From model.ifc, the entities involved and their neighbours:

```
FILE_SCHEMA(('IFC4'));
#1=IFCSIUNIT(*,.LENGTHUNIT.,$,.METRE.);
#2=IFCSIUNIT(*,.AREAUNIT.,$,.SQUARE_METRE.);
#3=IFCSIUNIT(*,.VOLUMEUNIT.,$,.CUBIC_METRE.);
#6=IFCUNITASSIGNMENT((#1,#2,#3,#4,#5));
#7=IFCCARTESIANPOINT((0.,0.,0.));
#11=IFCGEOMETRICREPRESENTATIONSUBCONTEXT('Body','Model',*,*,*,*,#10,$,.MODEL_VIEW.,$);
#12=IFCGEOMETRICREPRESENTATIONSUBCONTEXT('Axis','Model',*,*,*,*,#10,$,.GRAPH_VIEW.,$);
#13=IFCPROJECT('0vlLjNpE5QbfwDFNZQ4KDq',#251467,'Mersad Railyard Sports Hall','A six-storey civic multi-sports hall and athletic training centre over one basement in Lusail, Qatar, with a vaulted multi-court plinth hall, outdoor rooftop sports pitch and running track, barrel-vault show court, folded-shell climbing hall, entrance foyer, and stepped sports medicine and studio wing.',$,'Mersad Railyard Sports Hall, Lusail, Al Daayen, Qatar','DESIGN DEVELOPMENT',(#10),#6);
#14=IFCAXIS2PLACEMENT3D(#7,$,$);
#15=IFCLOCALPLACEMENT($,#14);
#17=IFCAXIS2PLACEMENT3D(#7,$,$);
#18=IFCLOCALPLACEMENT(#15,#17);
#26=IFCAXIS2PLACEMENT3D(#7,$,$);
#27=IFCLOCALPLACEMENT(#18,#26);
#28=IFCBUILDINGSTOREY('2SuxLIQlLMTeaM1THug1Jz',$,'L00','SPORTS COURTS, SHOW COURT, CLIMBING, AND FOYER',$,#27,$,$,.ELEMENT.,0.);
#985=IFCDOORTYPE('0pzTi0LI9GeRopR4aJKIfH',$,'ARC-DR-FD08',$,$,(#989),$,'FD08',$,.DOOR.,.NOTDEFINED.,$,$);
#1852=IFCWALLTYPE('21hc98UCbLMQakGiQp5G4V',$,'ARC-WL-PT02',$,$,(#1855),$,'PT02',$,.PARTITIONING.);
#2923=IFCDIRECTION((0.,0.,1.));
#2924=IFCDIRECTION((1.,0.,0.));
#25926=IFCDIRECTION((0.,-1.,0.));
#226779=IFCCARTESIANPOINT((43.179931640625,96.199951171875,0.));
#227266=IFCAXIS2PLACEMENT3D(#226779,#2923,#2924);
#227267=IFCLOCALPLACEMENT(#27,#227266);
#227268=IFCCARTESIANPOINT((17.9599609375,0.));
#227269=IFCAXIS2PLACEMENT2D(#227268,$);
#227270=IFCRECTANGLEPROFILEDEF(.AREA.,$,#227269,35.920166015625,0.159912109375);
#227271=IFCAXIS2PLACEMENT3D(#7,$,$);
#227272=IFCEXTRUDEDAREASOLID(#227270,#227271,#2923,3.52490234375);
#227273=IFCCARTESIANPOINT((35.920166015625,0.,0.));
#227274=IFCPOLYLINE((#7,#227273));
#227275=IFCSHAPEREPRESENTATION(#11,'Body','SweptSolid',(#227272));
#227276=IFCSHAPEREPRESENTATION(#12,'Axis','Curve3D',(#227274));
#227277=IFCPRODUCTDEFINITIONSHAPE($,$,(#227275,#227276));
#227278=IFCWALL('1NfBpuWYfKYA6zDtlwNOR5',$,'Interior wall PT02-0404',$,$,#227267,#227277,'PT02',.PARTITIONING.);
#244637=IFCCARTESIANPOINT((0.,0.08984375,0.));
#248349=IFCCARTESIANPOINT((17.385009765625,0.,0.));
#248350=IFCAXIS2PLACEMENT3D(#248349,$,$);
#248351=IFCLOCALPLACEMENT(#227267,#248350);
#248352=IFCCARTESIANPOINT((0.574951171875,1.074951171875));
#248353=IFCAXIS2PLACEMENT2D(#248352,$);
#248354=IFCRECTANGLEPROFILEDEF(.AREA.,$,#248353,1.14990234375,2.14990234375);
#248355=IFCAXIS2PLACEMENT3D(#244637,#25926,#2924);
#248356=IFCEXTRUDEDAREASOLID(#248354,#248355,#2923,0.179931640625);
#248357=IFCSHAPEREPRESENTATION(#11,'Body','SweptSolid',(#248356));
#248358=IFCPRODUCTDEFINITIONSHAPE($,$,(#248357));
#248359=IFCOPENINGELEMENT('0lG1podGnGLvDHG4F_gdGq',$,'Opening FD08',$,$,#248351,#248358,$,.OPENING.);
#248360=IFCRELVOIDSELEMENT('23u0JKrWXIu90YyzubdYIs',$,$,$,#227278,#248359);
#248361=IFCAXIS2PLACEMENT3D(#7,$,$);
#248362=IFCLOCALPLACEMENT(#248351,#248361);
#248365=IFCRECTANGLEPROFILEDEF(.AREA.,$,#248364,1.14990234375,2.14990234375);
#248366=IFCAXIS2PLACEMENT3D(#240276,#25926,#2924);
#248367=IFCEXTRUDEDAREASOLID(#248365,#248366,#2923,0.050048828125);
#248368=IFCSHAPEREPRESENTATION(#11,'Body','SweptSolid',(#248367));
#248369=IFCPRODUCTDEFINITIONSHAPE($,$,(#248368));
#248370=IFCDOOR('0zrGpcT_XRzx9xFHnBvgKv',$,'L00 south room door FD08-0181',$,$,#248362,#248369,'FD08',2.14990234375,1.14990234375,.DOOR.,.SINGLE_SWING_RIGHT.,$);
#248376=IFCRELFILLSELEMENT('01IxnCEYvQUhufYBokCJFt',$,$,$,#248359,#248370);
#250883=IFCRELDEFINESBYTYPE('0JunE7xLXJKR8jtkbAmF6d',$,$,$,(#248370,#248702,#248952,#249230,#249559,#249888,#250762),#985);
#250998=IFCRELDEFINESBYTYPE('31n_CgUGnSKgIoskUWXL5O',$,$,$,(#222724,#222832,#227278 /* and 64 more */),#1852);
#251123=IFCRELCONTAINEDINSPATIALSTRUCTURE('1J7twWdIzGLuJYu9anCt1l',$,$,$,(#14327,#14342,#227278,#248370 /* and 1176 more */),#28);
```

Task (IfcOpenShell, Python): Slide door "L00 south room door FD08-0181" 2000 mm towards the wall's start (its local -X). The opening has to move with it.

```python
import ifcopenshell
import ifcopenshell.api.geometry
import ifcopenshell.util.placement
import ifcopenshell.util.unit

model = ifcopenshell.open("model.ifc")
unit_scale = ifcopenshell.util.unit.calculate_unit_scale(model)

door = model.by_id(248370)
opening = door.FillsVoids[0].RelatingOpeningElement
wall = opening.VoidsElements[0].RelatingBuildingElement

wall_matrix = ifcopenshell.util.placement.get_local_placement(wall.ObjectPlacement)
shift = wall_matrix[:3, 0] * -2 / unit_scale
before = ifcopenshell.util.placement.get_local_placement(door.ObjectPlacement)[:3, 3].copy()

# The door is placed relative to its opening, so it follows when the opening moves.
matrix = ifcopenshell.util.placement.get_local_placement(opening.ObjectPlacement)
matrix[:3, 3] += shift
ifcopenshell.api.geometry.edit_object_placement(
    model, product=opening, matrix=matrix, is_si=False, should_transform_children=True
)

after = ifcopenshell.util.placement.get_local_placement(door.ObjectPlacement)[:3, 3]
print("door moved by", (after - before).round(3) + 0.0)

model.write("model_rev.ifc")
```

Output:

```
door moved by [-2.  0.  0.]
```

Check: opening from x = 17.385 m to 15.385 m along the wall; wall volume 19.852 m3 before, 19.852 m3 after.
